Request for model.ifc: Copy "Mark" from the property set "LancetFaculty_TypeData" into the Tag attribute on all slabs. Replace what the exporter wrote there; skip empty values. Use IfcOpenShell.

First a look at what the model holds.

```python
import ifcopenshell
import ifcopenshell.util.element

model = ifcopenshell.open("model.ifc")
print(model.schema)
slabs = model.by_type("IfcSlab")
print(len(slabs), "slabs")
for e in slabs[:8]:
    source = ifcopenshell.util.element.get_pset(e, "LancetFaculty_TypeData", "Mark")
    target = e.Tag
    print(e.id(), repr(source), repr(target), sep=" | ")
```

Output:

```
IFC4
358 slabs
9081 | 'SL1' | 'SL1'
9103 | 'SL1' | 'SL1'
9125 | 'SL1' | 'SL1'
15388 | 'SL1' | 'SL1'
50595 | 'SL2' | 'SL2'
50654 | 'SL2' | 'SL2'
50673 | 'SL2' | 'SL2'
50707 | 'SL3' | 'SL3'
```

```python
import ifcopenshell
import ifcopenshell.util.element

model = ifcopenshell.open("model.ifc")

count = 0
for e in model.by_type("IfcSlab"):
    value = ifcopenshell.util.element.get_pset(e, "LancetFaculty_TypeData", "Mark")
    current = e.Tag
    if not value or not value.strip() or current == value:
        continue
    e.Tag = value
    count += 1

print(count, "slabs updated")

model.write("model_v2.ifc")
```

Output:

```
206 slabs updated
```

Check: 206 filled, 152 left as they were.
